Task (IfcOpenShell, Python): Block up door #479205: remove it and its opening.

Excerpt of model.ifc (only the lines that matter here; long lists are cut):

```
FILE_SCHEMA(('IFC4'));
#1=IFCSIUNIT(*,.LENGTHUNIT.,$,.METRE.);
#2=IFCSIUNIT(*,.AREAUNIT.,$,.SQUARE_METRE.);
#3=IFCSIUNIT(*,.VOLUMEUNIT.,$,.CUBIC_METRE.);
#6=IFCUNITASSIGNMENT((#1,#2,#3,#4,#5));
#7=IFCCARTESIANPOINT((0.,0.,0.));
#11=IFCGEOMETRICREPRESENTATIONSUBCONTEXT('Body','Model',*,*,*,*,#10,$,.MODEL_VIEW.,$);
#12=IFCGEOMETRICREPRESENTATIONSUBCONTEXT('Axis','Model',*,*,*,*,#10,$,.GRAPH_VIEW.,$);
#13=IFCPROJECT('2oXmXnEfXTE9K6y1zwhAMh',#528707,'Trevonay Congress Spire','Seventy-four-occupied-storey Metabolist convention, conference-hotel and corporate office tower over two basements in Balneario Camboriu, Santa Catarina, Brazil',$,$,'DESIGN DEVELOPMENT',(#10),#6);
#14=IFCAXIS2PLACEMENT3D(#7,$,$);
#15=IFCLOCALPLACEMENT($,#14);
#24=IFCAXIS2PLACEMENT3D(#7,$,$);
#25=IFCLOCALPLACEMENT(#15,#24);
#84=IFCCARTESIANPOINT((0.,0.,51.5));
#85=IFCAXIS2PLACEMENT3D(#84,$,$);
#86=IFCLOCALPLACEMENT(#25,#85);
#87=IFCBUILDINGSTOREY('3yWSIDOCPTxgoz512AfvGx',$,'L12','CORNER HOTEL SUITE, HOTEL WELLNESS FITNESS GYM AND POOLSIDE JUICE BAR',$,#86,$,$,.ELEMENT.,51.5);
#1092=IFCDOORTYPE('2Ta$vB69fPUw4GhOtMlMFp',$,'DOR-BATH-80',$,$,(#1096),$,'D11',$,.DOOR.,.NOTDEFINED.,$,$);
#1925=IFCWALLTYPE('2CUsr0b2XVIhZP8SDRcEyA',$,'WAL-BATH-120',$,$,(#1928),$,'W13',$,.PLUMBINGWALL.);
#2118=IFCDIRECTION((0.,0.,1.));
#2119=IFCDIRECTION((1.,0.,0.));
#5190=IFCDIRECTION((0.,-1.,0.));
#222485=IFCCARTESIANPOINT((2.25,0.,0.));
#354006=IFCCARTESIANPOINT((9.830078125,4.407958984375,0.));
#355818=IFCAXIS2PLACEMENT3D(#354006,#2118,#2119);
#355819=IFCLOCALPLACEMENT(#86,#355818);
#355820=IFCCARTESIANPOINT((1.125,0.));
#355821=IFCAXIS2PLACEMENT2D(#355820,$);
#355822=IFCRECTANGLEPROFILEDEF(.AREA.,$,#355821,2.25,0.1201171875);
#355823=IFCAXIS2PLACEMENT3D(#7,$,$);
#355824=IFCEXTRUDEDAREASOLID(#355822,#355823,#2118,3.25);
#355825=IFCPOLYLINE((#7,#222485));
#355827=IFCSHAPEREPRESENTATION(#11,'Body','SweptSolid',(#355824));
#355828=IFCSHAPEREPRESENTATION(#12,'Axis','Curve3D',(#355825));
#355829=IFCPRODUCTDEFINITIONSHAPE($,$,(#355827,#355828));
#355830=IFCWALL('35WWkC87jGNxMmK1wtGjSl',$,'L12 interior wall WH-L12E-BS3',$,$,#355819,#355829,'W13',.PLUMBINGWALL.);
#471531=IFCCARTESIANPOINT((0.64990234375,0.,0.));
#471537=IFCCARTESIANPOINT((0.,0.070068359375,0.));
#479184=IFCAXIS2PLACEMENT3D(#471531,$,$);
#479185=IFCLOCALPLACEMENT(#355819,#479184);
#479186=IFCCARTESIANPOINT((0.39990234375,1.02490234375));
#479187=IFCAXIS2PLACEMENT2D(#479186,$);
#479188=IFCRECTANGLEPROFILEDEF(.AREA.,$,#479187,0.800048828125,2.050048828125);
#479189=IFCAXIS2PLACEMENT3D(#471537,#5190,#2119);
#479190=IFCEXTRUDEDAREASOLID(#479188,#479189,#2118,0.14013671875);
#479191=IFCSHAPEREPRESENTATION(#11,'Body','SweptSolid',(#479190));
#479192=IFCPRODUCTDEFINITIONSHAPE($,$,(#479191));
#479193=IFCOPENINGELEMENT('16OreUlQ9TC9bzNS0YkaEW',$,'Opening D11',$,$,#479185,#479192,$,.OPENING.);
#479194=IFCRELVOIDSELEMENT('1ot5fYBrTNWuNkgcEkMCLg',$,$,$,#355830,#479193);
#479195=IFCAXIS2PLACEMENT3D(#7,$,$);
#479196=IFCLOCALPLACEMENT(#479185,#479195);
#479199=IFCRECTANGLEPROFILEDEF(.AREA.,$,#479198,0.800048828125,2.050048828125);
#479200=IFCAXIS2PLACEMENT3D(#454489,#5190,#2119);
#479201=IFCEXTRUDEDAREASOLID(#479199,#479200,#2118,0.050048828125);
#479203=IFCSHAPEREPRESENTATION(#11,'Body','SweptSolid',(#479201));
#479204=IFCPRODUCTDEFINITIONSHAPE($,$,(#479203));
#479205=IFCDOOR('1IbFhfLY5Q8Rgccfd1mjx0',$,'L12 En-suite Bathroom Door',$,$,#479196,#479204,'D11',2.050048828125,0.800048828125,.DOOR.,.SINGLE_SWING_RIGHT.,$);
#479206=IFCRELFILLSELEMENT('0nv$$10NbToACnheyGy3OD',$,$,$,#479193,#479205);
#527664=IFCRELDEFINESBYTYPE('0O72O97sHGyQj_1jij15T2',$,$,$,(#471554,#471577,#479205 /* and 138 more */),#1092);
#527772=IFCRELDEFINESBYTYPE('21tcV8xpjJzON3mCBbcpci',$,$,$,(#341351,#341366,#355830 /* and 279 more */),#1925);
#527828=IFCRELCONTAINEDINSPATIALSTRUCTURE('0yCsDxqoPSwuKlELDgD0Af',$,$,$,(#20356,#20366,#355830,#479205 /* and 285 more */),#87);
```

```python
import ifcopenshell
import ifcopenshell.api.feature
import ifcopenshell.api.root
import ifcopenshell.geom
import ifcopenshell.util.shape

model = ifcopenshell.open("model.ifc")
settings = ifcopenshell.geom.settings()


def volume(element):
    """Net volume in cubic metres, openings subtracted."""
    shape = ifcopenshell.geom.create_shape(settings, element)
    return ifcopenshell.util.shape.get_volume(shape.geometry)


door = model.by_id(479205)
opening = door.FillsVoids[0].RelatingOpeningElement
wall = opening.VoidsElements[0].RelatingBuildingElement
before = volume(wall)

ifcopenshell.api.root.remove_product(model, product=door)
ifcopenshell.api.feature.remove_feature(model, feature=opening)

after = volume(wall)

print(f"wall volume {before:.3f} -> {after:.3f} m3")

model.write("model_updated.ifc")
```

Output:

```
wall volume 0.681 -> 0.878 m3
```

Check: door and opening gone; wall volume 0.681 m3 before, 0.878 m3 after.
